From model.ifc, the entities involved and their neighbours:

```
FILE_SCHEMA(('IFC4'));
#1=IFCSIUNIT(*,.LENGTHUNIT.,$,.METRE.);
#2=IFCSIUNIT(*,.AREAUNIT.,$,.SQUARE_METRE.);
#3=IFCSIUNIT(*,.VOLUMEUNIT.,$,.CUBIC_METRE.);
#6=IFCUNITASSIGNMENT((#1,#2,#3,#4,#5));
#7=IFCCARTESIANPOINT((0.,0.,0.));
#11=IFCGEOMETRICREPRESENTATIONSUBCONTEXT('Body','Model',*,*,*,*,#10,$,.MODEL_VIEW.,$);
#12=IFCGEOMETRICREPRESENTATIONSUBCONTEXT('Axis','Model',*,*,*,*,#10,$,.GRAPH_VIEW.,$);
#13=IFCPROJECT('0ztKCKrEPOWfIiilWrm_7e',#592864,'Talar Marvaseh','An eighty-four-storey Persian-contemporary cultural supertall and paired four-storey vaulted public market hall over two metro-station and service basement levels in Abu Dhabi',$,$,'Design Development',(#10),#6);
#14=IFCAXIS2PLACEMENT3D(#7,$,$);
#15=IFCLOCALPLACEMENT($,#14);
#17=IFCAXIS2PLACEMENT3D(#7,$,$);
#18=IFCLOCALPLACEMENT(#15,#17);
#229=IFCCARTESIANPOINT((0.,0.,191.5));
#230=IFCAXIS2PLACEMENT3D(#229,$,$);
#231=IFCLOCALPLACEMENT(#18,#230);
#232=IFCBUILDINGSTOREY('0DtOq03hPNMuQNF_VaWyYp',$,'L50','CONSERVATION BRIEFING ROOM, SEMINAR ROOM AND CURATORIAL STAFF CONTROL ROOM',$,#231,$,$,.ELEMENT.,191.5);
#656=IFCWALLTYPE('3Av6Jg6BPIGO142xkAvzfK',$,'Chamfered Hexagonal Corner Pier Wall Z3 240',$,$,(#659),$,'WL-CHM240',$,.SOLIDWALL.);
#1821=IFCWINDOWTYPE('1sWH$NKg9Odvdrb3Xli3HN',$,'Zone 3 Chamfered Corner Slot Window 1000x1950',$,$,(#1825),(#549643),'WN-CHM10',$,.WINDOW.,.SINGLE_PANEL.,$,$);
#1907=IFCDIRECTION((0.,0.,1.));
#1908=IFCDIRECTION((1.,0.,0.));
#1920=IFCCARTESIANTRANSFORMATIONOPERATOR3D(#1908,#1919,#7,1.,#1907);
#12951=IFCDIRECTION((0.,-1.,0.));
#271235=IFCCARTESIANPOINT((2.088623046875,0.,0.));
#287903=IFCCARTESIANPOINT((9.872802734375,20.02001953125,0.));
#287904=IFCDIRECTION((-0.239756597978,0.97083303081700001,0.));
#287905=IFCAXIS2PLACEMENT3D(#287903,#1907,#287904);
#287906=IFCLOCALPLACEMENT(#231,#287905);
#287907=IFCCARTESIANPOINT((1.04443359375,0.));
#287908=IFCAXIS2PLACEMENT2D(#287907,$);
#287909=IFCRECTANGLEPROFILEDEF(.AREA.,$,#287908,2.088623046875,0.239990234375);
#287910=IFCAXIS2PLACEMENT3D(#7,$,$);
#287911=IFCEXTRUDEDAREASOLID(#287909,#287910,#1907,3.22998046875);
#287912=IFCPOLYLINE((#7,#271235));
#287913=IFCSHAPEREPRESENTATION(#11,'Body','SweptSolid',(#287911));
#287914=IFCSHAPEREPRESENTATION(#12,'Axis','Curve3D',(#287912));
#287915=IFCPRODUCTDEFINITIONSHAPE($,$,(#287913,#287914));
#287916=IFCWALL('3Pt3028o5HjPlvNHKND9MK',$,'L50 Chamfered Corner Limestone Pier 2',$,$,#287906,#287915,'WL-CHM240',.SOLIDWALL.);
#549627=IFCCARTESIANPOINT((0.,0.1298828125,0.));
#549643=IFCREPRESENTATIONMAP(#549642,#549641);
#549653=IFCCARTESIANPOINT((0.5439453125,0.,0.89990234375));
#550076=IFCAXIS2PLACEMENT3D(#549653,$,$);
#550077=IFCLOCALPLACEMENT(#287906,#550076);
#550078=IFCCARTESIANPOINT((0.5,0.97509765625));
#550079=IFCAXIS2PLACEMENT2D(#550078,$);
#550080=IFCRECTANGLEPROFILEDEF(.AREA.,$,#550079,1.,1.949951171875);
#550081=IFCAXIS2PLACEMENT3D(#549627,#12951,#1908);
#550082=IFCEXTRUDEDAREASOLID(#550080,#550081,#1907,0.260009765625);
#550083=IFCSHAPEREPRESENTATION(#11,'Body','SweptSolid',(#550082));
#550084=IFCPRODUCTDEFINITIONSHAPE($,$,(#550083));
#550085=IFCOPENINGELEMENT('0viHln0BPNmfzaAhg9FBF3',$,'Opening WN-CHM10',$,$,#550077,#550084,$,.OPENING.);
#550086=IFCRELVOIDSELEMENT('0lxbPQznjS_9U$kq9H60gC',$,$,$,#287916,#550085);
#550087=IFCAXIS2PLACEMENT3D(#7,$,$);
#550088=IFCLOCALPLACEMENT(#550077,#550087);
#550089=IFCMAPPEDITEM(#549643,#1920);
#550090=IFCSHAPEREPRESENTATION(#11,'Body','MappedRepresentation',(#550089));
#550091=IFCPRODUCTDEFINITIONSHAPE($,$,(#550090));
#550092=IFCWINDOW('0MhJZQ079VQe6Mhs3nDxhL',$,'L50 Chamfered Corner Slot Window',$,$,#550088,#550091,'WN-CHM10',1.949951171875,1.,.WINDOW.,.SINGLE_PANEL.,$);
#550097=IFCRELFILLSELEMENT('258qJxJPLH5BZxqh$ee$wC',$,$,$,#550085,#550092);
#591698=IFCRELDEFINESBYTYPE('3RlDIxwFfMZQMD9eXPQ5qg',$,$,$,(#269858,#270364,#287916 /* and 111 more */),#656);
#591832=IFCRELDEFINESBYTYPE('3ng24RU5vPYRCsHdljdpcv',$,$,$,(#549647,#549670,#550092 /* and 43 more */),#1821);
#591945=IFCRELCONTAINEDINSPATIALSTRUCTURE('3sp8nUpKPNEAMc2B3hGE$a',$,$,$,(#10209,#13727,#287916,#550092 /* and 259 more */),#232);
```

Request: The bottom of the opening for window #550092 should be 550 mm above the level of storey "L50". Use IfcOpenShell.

```python
import numpy as np
import ifcopenshell
import ifcopenshell.api.geometry
import ifcopenshell.geom
import ifcopenshell.util.element
import ifcopenshell.util.placement
import ifcopenshell.util.shape
import ifcopenshell.util.unit

model = ifcopenshell.open("model.ifc")
unit_scale = ifcopenshell.util.unit.calculate_unit_scale(model)

window = model.by_guid("0MhJZQ079VQe6Mhs3nDxhL")
opening = window.FillsVoids[0].RelatingOpeningElement
storey = ifcopenshell.util.element.get_container(window, ifc_class="IfcBuildingStorey")
level = ifcopenshell.util.placement.get_local_placement(storey.ObjectPlacement)[2, 3]

# The opening's origin need not be at the sill, so measure its lowest point.
shape = ifcopenshell.geom.create_shape(ifcopenshell.geom.settings(), opening)
bottom = ifcopenshell.util.shape.get_shape_bottom_elevation(shape, shape.geometry) / unit_scale
dz = level + 0.55 - bottom

shift = np.array([0.0, 0.0, dz])
# The window is placed relative to its opening, so it follows when the opening moves.
matrix = ifcopenshell.util.placement.get_local_placement(opening.ObjectPlacement)
matrix[:3, 3] += shift
ifcopenshell.api.geometry.edit_object_placement(
    model, product=opening, matrix=matrix, is_si=False, should_transform_children=True
)

print(f"moved by {dz * unit_scale:+.3f} m")

model.write("model_rev.ifc")
```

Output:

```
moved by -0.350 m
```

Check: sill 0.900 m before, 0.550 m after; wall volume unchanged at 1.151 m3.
